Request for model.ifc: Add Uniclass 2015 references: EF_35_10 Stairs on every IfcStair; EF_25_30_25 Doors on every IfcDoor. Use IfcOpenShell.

First a look at what the model holds.

```python
import ifcopenshell

model = ifcopenshell.open("model.ifc")
print(model.schema)
print("classifications:", [c.Name for c in model.by_type("IfcClassification")])
for ifc_class in ("IfcDoor", "IfcRoof", "IfcStair", "IfcWall", "IfcWindow"):
    print(ifc_class, len(model.by_type(ifc_class)))
```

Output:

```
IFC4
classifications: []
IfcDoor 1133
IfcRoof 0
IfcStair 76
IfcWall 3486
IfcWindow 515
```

```python
import ifcopenshell
import ifcopenshell.api.classification

model = ifcopenshell.open("model.ifc")

system = ifcopenshell.api.classification.add_classification(model, classification="Uniclass 2015")

codes = {
    "IfcStair": ("EF_35_10", "Stairs"),
    "IfcDoor": ("EF_25_30_25", "Doors"),
}
for ifc_class, (code, name) in codes.items():
    products = model.by_type(ifc_class)
    ifcopenshell.api.classification.add_reference(
        model, products=products, classification=system, identification=code, name=name
    )
    print(code, len(products))

model.write("model_updated.ifc")
```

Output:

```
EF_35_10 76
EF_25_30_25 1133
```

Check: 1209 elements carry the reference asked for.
